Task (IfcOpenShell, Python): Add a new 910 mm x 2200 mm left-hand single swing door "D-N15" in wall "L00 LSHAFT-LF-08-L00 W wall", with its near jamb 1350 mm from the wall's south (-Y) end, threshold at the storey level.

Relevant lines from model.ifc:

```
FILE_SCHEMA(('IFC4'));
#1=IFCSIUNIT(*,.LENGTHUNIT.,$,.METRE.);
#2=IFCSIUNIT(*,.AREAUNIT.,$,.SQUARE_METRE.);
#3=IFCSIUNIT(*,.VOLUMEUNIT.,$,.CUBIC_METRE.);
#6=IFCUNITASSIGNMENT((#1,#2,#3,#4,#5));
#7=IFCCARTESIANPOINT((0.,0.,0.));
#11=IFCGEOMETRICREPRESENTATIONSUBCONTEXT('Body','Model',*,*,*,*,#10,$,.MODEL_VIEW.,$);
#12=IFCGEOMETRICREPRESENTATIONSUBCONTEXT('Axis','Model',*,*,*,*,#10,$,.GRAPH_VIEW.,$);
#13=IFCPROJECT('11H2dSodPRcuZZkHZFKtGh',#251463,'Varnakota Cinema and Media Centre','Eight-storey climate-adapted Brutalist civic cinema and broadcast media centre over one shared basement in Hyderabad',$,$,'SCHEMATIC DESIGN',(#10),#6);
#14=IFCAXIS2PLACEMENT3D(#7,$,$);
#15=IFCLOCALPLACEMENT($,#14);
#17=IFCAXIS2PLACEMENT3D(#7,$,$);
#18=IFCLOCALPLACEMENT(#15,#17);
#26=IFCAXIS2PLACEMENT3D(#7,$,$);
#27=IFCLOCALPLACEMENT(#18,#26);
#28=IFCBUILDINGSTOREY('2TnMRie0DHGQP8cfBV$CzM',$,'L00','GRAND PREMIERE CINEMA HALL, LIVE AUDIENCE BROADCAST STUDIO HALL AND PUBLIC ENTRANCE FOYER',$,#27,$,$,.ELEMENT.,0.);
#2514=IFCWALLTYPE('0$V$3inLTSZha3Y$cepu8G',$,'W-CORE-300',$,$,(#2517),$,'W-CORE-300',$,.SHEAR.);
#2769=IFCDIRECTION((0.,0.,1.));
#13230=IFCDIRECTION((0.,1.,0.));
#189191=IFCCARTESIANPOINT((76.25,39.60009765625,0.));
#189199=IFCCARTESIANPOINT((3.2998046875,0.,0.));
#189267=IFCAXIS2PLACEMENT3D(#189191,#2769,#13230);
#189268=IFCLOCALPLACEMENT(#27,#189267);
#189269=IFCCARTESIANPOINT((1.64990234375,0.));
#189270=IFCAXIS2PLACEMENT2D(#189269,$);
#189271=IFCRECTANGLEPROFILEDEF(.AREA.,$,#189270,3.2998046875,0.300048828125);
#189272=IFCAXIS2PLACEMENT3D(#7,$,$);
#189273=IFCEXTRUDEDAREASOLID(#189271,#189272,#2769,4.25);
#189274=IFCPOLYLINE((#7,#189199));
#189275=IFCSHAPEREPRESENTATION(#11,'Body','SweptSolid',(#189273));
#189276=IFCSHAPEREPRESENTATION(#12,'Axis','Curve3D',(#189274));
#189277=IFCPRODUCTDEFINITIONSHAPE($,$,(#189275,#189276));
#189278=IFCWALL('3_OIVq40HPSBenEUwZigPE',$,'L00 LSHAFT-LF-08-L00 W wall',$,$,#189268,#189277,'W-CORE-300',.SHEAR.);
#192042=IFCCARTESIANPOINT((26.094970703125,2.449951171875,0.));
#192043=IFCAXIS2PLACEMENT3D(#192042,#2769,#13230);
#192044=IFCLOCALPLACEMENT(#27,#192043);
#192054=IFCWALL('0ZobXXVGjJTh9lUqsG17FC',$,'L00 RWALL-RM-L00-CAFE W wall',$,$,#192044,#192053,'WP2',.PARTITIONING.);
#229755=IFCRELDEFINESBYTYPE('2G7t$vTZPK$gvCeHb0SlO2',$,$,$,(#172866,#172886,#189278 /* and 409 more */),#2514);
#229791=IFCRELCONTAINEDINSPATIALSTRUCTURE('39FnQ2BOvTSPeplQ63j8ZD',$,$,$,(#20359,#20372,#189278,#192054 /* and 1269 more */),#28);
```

```python
import numpy as np
import ifcopenshell
import ifcopenshell.api.feature
import ifcopenshell.api.geometry
import ifcopenshell.api.root
import ifcopenshell.api.spatial
import ifcopenshell.geom
import ifcopenshell.util.element
import ifcopenshell.util.placement
import ifcopenshell.util.representation
import ifcopenshell.util.shape
import ifcopenshell.util.unit

model = ifcopenshell.open("model.ifc")
unit_scale = ifcopenshell.util.unit.calculate_unit_scale(model)
settings = ifcopenshell.geom.settings()


def volume(element):
    """Net volume in cubic metres, openings subtracted."""
    shape = ifcopenshell.geom.create_shape(settings, element)
    return ifcopenshell.util.shape.get_volume(shape.geometry)


wall = model.by_id(189278)
storey = ifcopenshell.util.element.get_container(wall, ifc_class="IfcBuildingStorey")
context = ifcopenshell.util.representation.get_context(model, "Model", "Body", "MODEL_VIEW")
before = volume(wall)

width, height, from_end, sill = 0.91, 2.2, 1.35, 0.0  # metres

# The wall runs along its own X axis, and the end named is its -X end.
wall_shape = ifcopenshell.geom.create_shape(settings, wall)
x, y, z = ifcopenshell.util.shape.get_vertices(wall_shape.geometry).T
start = x.min() + from_end
face, thickness = float(y.min()), float(y.max() - y.min())
wall_matrix = ifcopenshell.util.placement.get_local_placement(wall.ObjectPlacement)
level = ifcopenshell.util.placement.get_local_placement(storey.ObjectPlacement)[2, 3]


def in_wall(x, y):
    """Placement at x, y metres in the wall's axes, at sill height."""
    matrix = wall_matrix.copy()
    matrix[:, 3] = wall_matrix @ np.array([x / unit_scale, y / unit_scale, 0.0, 1.0])
    matrix[2, 3] = level + sill / unit_scale
    return matrix


# Opening: a box that overshoots both wall faces by 50 mm.
opening = ifcopenshell.api.root.create_entity(model, ifc_class="IfcOpeningElement", predefined_type="OPENING")
box = ifcopenshell.api.geometry.add_wall_representation(
    model, context=context, length=width, height=height, thickness=thickness + 0.1
)
ifcopenshell.api.geometry.assign_representation(model, product=opening, representation=box)
ifcopenshell.api.geometry.edit_object_placement(model, product=opening, matrix=in_wall(start, face - 0.05), is_si=False)
ifcopenshell.api.feature.add_feature(model, feature=opening, element=wall)

door = ifcopenshell.api.root.create_entity(model, ifc_class="IfcDoor", name="D-N15", predefined_type="DOOR")
door.OverallWidth, door.OverallHeight = width / unit_scale, height / unit_scale
door.OperationType = "SINGLE_SWING_LEFT"
body = ifcopenshell.api.geometry.add_door_representation(
    model,
    context=context,
    overall_width=door.OverallWidth,
    overall_height=door.OverallHeight,
    operation_type="SINGLE_SWING_LEFT",
    lining_properties={"LiningDepth": thickness / unit_scale, "ThresholdDepth": thickness / unit_scale},
)
ifcopenshell.api.geometry.assign_representation(model, product=door, representation=body)
ifcopenshell.api.spatial.assign_container(model, products=[door], relating_structure=storey)
ifcopenshell.api.feature.add_filling(model, opening=opening, element=door)

# The lining spans the wall, so the door starts at the wall face.
ifcopenshell.api.geometry.edit_object_placement(model, product=door, matrix=in_wall(start, face), is_si=False)

after = volume(wall)

print(f"wall volume {before:.3f} -> {after:.3f} m3")

model.write("model_v2.ifc")
```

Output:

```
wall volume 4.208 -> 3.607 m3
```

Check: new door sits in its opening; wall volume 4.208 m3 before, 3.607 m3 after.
